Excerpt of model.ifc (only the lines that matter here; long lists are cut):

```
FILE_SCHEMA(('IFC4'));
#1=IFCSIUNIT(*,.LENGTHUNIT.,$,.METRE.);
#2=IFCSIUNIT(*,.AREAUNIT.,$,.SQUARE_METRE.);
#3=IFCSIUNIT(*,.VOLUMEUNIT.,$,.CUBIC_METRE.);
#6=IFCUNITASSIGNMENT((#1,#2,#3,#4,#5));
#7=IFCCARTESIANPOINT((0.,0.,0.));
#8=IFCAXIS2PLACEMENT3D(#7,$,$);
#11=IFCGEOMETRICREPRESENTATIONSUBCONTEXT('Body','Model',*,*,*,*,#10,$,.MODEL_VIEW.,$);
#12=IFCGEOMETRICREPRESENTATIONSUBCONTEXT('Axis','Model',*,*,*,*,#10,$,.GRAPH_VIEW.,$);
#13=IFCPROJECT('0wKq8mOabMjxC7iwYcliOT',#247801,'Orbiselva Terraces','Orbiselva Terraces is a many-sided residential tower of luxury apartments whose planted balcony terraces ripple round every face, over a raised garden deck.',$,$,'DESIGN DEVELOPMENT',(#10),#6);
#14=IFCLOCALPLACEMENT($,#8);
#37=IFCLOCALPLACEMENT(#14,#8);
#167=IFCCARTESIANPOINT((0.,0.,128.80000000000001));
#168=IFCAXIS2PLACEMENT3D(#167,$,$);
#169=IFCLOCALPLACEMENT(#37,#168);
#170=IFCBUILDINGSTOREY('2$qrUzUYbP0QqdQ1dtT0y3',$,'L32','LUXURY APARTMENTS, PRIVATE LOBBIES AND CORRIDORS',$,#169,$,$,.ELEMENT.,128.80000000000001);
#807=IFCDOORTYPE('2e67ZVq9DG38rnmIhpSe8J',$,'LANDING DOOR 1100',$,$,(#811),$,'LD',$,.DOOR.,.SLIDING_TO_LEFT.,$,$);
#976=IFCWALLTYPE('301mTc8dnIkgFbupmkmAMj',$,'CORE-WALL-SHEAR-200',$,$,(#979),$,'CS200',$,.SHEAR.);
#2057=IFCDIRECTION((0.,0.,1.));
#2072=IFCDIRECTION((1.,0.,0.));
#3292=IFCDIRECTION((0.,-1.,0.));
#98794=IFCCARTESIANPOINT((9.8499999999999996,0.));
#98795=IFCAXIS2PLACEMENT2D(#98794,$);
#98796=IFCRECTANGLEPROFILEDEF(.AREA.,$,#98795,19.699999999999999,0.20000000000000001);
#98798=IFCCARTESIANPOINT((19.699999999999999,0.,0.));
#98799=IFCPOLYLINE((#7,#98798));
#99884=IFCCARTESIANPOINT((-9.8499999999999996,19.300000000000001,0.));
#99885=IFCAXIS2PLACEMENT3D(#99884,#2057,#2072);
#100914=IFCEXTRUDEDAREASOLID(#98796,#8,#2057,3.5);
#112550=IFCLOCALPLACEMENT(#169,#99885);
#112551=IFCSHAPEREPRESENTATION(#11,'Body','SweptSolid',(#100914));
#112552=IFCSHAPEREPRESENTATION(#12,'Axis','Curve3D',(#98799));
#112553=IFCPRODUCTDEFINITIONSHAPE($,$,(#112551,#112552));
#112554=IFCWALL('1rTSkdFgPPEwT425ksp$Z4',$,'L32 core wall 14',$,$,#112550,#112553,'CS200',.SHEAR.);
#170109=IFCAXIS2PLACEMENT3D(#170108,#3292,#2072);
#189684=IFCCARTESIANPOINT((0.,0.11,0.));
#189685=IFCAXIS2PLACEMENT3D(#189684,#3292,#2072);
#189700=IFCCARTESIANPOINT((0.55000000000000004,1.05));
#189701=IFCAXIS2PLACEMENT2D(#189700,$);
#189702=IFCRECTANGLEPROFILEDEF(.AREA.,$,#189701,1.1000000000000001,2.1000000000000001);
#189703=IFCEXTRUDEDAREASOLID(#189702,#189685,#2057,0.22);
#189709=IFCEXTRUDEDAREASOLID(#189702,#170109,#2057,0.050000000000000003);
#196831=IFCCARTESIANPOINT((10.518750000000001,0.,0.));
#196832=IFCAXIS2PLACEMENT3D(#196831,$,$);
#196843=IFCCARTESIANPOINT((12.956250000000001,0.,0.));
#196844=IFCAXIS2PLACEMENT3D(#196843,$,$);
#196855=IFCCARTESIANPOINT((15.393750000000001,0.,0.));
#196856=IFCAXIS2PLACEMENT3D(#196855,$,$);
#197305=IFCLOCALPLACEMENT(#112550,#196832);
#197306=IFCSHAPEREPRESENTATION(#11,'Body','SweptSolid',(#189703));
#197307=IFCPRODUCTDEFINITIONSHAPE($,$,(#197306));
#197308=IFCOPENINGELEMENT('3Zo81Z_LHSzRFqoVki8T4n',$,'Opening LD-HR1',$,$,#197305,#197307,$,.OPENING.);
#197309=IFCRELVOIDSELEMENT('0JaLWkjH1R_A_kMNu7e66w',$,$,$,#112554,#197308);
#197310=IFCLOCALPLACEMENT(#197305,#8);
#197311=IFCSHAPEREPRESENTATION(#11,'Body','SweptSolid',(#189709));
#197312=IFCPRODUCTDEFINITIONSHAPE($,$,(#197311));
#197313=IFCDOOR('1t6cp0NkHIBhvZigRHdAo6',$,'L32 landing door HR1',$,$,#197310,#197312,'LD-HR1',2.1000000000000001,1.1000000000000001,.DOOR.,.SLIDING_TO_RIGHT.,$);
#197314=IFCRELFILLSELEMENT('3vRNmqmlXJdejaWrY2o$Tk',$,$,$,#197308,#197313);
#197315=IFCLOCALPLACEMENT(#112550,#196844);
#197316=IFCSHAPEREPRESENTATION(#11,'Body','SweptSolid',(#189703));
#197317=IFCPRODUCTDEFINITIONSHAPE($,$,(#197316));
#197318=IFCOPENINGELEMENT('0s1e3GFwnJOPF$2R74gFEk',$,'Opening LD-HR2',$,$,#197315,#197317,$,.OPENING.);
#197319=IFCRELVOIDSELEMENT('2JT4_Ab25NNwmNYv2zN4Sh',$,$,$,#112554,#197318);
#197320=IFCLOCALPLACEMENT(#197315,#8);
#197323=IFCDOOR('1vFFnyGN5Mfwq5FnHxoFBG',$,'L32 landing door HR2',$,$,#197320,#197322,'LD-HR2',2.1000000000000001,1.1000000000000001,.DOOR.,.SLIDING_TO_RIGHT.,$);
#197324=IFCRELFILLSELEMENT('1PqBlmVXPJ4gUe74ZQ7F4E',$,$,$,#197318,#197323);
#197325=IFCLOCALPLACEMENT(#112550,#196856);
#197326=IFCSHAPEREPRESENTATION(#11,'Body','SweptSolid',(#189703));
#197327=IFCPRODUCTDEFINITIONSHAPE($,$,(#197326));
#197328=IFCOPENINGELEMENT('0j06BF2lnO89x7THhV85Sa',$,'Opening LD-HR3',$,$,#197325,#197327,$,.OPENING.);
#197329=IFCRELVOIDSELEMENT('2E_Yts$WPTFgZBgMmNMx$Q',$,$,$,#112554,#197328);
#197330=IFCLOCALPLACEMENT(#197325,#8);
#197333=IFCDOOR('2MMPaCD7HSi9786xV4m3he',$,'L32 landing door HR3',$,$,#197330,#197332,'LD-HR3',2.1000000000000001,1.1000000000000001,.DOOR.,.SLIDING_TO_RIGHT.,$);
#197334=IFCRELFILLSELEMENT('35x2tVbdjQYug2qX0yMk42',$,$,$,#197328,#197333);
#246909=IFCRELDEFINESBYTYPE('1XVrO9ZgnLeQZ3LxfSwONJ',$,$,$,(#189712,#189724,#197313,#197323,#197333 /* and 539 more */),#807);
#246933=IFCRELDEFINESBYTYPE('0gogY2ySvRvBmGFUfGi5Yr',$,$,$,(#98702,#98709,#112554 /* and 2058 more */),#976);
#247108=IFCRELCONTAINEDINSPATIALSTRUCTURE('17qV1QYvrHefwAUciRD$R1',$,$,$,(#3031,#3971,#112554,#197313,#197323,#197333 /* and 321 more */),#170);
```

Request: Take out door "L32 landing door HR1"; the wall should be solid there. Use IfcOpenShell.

```python
import ifcopenshell
import ifcopenshell.api.feature
import ifcopenshell.api.root
import ifcopenshell.geom
import ifcopenshell.util.shape

model = ifcopenshell.open("model.ifc")
settings = ifcopenshell.geom.settings()


def volume(element):
    """Net volume in cubic metres, openings subtracted."""
    shape = ifcopenshell.geom.create_shape(settings, element)
    return ifcopenshell.util.shape.get_volume(shape.geometry)


door = model.by_guid("1t6cp0NkHIBhvZigRHdAo6")
opening = door.FillsVoids[0].RelatingOpeningElement
wall = opening.VoidsElements[0].RelatingBuildingElement
before = volume(wall)

ifcopenshell.api.root.remove_product(model, product=door)
ifcopenshell.api.feature.remove_feature(model, feature=opening)

after = volume(wall)

print(f"wall volume {before:.3f} -> {after:.3f} m3")

model.write("model-out.ifc")
```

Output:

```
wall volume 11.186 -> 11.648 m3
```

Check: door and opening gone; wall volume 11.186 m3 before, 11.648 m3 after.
